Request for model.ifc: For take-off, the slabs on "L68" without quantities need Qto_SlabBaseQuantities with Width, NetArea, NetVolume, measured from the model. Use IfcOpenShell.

First a look at what the model holds.

```python
import ifcopenshell
import ifcopenshell.util.element
import ifcopenshell.util.unit

model = ifcopenshell.open("model.ifc")
print(model.schema)
for unit_type in ("LENGTHUNIT", "AREAUNIT", "VOLUMEUNIT"):
    print(unit_type, ifcopenshell.util.unit.calculate_unit_scale(model, unit_type))
storey = next(s for s in model.by_type("IfcBuildingStorey") if s.Name == "L68")
slabs = [e for e in ifcopenshell.util.element.get_decomposition(storey) if e.is_a("IfcSlab")]
for e in sorted(slabs, key=lambda e: e.id()):
    print(e.id(), e.is_a(), e.Name, list(ifcopenshell.util.element.get_psets(e, qtos_only=True)), sep=" | ")
```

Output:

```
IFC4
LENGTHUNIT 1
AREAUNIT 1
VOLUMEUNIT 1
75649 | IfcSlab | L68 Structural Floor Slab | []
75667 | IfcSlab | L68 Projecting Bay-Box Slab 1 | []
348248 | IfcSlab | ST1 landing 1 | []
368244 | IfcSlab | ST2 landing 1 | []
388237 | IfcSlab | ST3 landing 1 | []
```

```python
import ifcopenshell
import ifcopenshell.api.pset
import ifcopenshell.geom
import ifcopenshell.util.element
import ifcopenshell.util.shape
import ifcopenshell.util.unit

model = ifcopenshell.open("model.ifc")
unit_scale = ifcopenshell.util.unit.calculate_unit_scale(model)
area_scale = ifcopenshell.util.unit.calculate_unit_scale(model, "AREAUNIT")
volume_scale = ifcopenshell.util.unit.calculate_unit_scale(model, "VOLUMEUNIT")
settings = ifcopenshell.geom.settings()

storey = next(s for s in model.by_type("IfcBuildingStorey") if s.Name == "L68")
slabs = [e for e in ifcopenshell.util.element.get_decomposition(storey) if e.is_a("IfcSlab")]

for e in sorted(slabs, key=lambda e: e.id()):
    if ifcopenshell.util.element.get_psets(e, qtos_only=True, should_inherit=False):
        continue
    # Geometry comes back in metres, in the element's own axes.
    shape = ifcopenshell.geom.create_shape(settings, e)
    values = {
        "Width": ifcopenshell.util.shape.get_z(shape.geometry) / unit_scale,
        "NetArea": ifcopenshell.util.shape.get_footprint_area(shape.geometry) / area_scale,
        "NetVolume": ifcopenshell.util.shape.get_volume(shape.geometry) / volume_scale,
    }
    qto = ifcopenshell.api.pset.add_qto(model, product=e, name="Qto_SlabBaseQuantities")
    ifcopenshell.api.pset.edit_qto(model, qto=qto, properties=values)
    print(e.id(), {k: round(v, 3) for k, v in values.items()})

model.write("model_updated.ifc")
```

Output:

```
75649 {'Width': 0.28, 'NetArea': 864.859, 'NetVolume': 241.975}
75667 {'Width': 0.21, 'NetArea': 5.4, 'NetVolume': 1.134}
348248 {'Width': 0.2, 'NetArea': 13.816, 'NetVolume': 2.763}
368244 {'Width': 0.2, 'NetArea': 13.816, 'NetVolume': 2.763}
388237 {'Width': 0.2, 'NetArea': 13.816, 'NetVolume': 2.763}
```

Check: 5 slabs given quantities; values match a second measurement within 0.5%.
